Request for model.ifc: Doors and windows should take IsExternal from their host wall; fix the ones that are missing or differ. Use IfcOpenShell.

First a look at what the model holds.

```python
import ifcopenshell
import ifcopenshell.util.element

model = ifcopenshell.open("model.ifc")
print(model.schema)
seen = {}
for e in model.by_type("IfcDoor") + model.by_type("IfcWindow"):
    if not e.FillsVoids:
        continue
    host = e.FillsVoids[0].RelatingOpeningElement.VoidsElements[0].RelatingBuildingElement
    own = ifcopenshell.util.element.get_pset(e, f"Pset_{e.is_a()[3:].removesuffix('StandardCase')}Common", "IsExternal")
    wall = ifcopenshell.util.element.get_pset(host, "Pset_WallCommon", "IsExternal")
    seen[e.is_a(), own, wall] = seen.get((e.is_a(), own, wall), 0) + 1
for (cls, own, wall), count in sorted(seen.items(), key=str):
    print(count, cls, "IsExternal:", own, "| host wall:", wall)
```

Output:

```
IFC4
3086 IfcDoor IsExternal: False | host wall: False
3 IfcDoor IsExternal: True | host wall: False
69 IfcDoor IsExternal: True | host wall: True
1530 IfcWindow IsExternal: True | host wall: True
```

```python
import ifcopenshell
import ifcopenshell.api.pset
import ifcopenshell.util.element

model = ifcopenshell.open("model.ifc")

count = 0
for ifc_class, pset_name in (("IfcDoor", "Pset_DoorCommon"), ("IfcWindow", "Pset_WindowCommon")):
    for e in model.by_type(ifc_class):
        if not e.FillsVoids:
            continue
        host = e.FillsVoids[0].RelatingOpeningElement.VoidsElements[0].RelatingBuildingElement
        external = ifcopenshell.util.element.get_pset(host, "Pset_WallCommon", "IsExternal")
        if external is None or ifcopenshell.util.element.get_pset(e, pset_name, "IsExternal") == external:
            continue
        found = ifcopenshell.util.element.get_pset(e, pset_name, should_inherit=False)
        if found:
            pset = model.by_id(found["id"])
            if len(ifcopenshell.util.element.get_elements_by_pset(pset)) > 1:
                pset = ifcopenshell.api.pset.unshare_pset(model, products=[e], pset=pset)[0]
        else:
            pset = ifcopenshell.api.pset.add_pset(model, product=e, name=pset_name)
        ifcopenshell.api.pset.edit_pset(model, pset=pset, properties={"IsExternal": external})
        count += 1

print(count, "updated")

model.write("model_v2.ifc")
```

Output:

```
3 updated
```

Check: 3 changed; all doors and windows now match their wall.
